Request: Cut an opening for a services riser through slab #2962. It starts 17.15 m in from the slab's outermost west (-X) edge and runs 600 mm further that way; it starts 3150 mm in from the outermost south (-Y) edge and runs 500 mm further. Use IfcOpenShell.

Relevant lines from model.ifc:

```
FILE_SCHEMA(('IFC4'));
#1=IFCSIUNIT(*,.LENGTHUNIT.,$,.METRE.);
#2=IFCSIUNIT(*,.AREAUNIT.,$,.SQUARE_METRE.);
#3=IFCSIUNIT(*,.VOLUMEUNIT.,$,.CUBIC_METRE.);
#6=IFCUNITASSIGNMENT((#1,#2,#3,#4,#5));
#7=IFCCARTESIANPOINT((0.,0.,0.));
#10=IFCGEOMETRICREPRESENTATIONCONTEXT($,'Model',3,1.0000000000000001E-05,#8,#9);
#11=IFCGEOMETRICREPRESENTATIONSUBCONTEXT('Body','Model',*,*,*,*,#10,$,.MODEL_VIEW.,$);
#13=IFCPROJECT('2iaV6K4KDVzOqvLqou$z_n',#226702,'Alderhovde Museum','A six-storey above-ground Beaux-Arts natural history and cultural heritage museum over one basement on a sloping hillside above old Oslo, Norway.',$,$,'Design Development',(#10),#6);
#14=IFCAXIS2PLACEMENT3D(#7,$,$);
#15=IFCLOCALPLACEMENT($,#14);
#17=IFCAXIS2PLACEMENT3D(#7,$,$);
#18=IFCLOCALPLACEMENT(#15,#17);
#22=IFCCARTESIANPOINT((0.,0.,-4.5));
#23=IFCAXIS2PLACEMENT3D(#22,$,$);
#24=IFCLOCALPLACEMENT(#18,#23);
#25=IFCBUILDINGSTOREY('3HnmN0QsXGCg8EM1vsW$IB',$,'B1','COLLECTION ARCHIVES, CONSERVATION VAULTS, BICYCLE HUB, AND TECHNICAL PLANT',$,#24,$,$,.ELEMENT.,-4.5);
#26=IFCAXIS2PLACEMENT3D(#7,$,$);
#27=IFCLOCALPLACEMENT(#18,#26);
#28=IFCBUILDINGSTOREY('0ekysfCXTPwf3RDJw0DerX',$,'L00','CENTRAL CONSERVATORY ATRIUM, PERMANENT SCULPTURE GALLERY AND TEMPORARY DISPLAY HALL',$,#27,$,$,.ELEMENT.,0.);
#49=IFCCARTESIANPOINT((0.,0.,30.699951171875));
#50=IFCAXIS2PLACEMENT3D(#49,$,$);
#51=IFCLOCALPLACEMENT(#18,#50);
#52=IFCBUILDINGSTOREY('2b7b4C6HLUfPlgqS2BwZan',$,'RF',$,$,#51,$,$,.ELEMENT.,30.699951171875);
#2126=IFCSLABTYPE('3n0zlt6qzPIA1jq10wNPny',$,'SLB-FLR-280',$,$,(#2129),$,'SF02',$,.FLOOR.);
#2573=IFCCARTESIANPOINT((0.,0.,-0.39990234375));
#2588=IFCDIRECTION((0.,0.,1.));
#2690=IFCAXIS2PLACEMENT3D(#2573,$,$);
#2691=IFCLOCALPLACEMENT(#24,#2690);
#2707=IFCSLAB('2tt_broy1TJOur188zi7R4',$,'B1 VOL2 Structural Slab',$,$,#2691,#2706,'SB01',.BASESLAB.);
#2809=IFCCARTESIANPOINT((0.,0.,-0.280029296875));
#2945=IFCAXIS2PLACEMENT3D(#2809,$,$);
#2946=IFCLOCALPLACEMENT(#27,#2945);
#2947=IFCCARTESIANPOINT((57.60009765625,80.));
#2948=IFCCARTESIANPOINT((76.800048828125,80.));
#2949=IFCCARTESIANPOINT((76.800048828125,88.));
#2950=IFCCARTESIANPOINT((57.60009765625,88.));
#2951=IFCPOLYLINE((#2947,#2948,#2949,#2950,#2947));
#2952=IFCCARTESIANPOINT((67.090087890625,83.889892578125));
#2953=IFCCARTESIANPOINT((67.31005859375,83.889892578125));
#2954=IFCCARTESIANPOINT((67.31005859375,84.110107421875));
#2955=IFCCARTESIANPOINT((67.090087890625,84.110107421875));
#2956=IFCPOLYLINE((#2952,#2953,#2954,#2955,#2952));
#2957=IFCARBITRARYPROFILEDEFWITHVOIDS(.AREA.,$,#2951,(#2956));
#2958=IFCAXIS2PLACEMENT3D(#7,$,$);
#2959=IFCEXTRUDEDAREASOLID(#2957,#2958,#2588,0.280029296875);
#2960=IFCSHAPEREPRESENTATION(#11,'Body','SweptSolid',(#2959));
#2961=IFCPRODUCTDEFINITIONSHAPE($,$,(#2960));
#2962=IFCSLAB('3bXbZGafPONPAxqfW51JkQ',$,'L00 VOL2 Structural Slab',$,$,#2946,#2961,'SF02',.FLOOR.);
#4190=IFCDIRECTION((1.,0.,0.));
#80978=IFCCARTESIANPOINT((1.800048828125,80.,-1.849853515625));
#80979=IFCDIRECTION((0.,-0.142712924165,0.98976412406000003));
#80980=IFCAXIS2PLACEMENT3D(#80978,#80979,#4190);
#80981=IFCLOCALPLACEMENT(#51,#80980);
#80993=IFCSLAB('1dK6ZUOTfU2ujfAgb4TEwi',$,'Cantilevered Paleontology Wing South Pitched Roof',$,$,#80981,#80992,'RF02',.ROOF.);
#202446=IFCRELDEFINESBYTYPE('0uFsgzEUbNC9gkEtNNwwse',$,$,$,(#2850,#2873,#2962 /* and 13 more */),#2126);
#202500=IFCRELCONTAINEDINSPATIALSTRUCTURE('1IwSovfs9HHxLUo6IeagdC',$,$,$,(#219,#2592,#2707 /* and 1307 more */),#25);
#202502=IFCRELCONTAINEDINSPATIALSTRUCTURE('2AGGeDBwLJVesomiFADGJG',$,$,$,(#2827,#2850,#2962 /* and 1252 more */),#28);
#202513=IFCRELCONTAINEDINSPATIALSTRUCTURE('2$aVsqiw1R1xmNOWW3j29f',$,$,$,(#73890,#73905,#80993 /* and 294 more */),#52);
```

```python
import numpy as np
import ifcopenshell
import ifcopenshell.api.feature
import ifcopenshell.api.geometry
import ifcopenshell.api.root
import ifcopenshell.geom
import ifcopenshell.util.placement
import ifcopenshell.util.representation
import ifcopenshell.util.shape
import ifcopenshell.util.unit

model = ifcopenshell.open("model.ifc")
unit_scale = ifcopenshell.util.unit.calculate_unit_scale(model)
settings = ifcopenshell.geom.settings()


def volume(element):
    """Net volume in cubic metres, openings subtracted."""
    shape = ifcopenshell.geom.create_shape(settings, element)
    return ifcopenshell.util.shape.get_volume(shape.geometry)


slab = model.by_guid("3bXbZGafPONPAxqfW51JkQ")
before = volume(slab)

# Extent in the slab's own axes, in metres. The edges named are its -X and -Y sides.
slab_shape = ifcopenshell.geom.create_shape(settings, slab)
vertices = ifcopenshell.util.shape.get_vertices(slab_shape.geometry)
x_min, y_min, bottom = vertices.min(axis=0)
top = vertices[:, 2].max()

opening = ifcopenshell.api.root.create_entity(model, ifc_class="IfcOpeningElement", name="Services riser opening", predefined_type="OPENING")
context = ifcopenshell.util.representation.get_context(model, "Model", "Body", "MODEL_VIEW")
width, depth = 0.6, 0.5
outline = [(0.0, 0.0), (width, 0.0), (width, depth), (0.0, depth), (0.0, 0.0)]
# Overshoot both faces by 50 mm so the cut is clean.
shape = ifcopenshell.api.geometry.add_slab_representation(
    model, context=context, depth=top - bottom + 0.1, polyline=outline
)
ifcopenshell.api.geometry.assign_representation(model, product=opening, representation=shape)

matrix = ifcopenshell.util.placement.get_local_placement(slab.ObjectPlacement)
matrix[:, 3] = matrix @ np.append(np.array([x_min + 17.15, y_min + 3.15, bottom - 0.05]) / unit_scale, 1.0)
ifcopenshell.api.geometry.edit_object_placement(model, product=opening, matrix=matrix, is_si=False)
ifcopenshell.api.feature.add_feature(model, feature=opening, element=slab)

after = volume(slab)

print(f"slab volume {before:.3f} -> {after:.3f} m3")

model.write("model-out.ifc")
```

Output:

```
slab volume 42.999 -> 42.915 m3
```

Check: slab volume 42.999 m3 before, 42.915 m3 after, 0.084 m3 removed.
